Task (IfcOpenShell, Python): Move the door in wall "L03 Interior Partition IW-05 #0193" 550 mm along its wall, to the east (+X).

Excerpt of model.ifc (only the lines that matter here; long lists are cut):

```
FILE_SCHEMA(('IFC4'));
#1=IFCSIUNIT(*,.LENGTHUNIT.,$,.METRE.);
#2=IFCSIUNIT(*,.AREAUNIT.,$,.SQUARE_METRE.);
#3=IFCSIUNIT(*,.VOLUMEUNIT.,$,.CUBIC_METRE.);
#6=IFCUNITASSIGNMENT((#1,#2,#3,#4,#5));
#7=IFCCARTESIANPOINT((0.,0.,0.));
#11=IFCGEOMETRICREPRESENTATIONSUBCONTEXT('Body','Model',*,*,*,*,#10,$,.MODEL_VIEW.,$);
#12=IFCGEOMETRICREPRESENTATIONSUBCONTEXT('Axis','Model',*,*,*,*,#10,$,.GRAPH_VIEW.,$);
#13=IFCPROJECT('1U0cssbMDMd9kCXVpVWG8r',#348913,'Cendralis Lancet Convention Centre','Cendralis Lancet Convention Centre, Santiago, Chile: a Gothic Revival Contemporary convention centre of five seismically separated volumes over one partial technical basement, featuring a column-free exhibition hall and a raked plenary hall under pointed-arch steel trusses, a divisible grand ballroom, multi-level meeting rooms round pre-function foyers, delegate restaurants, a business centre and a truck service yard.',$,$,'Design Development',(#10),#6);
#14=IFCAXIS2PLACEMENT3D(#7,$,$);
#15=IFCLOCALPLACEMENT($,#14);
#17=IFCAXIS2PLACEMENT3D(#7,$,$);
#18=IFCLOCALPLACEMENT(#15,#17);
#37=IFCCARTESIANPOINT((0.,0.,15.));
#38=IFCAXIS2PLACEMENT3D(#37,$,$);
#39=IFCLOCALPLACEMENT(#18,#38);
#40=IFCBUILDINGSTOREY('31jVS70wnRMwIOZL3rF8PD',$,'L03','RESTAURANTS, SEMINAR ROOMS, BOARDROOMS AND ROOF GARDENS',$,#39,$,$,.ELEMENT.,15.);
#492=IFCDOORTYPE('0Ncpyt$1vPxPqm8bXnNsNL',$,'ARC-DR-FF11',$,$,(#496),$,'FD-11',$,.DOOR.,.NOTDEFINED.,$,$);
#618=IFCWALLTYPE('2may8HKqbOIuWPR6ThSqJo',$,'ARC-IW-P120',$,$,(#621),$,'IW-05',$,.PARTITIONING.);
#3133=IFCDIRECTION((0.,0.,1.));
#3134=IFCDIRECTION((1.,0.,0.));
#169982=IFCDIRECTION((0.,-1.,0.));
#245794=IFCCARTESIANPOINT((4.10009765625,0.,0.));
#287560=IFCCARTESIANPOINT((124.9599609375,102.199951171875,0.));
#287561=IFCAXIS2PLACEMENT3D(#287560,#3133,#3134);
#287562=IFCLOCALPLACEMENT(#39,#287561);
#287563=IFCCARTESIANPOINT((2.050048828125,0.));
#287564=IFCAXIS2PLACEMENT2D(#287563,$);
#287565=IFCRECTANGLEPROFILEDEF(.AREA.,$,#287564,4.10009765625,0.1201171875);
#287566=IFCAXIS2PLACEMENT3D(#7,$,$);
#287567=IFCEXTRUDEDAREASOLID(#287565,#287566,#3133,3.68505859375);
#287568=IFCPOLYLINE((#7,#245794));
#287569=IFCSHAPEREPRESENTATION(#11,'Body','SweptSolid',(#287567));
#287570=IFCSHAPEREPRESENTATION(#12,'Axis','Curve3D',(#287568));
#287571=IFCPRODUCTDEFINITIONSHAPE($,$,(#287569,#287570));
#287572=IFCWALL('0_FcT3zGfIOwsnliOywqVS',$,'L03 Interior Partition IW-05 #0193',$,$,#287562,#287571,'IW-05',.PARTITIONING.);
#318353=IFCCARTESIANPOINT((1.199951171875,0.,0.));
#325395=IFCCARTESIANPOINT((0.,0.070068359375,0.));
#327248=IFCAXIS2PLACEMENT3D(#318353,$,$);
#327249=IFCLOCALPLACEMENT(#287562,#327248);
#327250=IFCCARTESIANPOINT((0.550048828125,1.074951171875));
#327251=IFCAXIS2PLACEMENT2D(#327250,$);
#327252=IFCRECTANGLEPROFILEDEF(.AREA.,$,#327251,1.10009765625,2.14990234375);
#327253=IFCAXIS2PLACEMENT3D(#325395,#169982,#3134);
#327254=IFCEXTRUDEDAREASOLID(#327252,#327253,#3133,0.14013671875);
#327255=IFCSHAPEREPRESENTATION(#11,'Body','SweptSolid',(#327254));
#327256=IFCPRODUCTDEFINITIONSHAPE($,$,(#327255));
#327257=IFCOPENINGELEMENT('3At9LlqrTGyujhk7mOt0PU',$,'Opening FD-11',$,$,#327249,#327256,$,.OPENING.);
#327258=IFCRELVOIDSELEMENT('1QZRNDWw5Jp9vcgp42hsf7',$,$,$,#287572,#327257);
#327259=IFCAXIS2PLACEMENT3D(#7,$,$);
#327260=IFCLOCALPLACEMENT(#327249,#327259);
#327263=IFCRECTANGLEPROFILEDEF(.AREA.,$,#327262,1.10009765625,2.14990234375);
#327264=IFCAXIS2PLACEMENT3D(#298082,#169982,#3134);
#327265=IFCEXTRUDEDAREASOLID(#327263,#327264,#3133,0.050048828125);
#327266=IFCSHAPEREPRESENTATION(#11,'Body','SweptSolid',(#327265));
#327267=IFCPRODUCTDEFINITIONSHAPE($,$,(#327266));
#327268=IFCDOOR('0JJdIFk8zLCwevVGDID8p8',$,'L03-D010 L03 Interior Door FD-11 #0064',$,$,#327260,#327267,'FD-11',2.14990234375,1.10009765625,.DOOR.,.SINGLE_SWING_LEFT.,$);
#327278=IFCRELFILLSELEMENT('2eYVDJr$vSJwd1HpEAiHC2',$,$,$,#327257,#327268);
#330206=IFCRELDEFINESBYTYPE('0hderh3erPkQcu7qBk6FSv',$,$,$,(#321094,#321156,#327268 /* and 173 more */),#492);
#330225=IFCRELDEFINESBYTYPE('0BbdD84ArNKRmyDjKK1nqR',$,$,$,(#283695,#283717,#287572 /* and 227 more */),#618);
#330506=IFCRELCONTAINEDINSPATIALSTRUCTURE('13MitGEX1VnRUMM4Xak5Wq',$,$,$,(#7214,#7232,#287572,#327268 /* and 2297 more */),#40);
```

```python
import ifcopenshell
import ifcopenshell.api.geometry
import ifcopenshell.util.placement

model = ifcopenshell.open("model.ifc")

door = model.by_id(327268)
opening = door.FillsVoids[0].RelatingOpeningElement
wall = opening.VoidsElements[0].RelatingBuildingElement

wall_matrix = ifcopenshell.util.placement.get_local_placement(wall.ObjectPlacement)
shift = wall_matrix[:3, 0] * 0.55
before = ifcopenshell.util.placement.get_local_placement(door.ObjectPlacement)[:3, 3].copy()

# The door is placed relative to its opening, so it follows when the opening moves.
matrix = ifcopenshell.util.placement.get_local_placement(opening.ObjectPlacement)
matrix[:3, 3] += shift
ifcopenshell.api.geometry.edit_object_placement(
    model, product=opening, matrix=matrix, is_si=False, should_transform_children=True
)

after = ifcopenshell.util.placement.get_local_placement(door.ObjectPlacement)[:3, 3]
print("door moved by", (after - before).round(3) + 0.0)

model.write("model_v2.ifc")
```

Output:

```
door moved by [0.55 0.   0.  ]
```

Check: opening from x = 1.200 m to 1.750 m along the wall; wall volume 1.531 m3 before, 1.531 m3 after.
